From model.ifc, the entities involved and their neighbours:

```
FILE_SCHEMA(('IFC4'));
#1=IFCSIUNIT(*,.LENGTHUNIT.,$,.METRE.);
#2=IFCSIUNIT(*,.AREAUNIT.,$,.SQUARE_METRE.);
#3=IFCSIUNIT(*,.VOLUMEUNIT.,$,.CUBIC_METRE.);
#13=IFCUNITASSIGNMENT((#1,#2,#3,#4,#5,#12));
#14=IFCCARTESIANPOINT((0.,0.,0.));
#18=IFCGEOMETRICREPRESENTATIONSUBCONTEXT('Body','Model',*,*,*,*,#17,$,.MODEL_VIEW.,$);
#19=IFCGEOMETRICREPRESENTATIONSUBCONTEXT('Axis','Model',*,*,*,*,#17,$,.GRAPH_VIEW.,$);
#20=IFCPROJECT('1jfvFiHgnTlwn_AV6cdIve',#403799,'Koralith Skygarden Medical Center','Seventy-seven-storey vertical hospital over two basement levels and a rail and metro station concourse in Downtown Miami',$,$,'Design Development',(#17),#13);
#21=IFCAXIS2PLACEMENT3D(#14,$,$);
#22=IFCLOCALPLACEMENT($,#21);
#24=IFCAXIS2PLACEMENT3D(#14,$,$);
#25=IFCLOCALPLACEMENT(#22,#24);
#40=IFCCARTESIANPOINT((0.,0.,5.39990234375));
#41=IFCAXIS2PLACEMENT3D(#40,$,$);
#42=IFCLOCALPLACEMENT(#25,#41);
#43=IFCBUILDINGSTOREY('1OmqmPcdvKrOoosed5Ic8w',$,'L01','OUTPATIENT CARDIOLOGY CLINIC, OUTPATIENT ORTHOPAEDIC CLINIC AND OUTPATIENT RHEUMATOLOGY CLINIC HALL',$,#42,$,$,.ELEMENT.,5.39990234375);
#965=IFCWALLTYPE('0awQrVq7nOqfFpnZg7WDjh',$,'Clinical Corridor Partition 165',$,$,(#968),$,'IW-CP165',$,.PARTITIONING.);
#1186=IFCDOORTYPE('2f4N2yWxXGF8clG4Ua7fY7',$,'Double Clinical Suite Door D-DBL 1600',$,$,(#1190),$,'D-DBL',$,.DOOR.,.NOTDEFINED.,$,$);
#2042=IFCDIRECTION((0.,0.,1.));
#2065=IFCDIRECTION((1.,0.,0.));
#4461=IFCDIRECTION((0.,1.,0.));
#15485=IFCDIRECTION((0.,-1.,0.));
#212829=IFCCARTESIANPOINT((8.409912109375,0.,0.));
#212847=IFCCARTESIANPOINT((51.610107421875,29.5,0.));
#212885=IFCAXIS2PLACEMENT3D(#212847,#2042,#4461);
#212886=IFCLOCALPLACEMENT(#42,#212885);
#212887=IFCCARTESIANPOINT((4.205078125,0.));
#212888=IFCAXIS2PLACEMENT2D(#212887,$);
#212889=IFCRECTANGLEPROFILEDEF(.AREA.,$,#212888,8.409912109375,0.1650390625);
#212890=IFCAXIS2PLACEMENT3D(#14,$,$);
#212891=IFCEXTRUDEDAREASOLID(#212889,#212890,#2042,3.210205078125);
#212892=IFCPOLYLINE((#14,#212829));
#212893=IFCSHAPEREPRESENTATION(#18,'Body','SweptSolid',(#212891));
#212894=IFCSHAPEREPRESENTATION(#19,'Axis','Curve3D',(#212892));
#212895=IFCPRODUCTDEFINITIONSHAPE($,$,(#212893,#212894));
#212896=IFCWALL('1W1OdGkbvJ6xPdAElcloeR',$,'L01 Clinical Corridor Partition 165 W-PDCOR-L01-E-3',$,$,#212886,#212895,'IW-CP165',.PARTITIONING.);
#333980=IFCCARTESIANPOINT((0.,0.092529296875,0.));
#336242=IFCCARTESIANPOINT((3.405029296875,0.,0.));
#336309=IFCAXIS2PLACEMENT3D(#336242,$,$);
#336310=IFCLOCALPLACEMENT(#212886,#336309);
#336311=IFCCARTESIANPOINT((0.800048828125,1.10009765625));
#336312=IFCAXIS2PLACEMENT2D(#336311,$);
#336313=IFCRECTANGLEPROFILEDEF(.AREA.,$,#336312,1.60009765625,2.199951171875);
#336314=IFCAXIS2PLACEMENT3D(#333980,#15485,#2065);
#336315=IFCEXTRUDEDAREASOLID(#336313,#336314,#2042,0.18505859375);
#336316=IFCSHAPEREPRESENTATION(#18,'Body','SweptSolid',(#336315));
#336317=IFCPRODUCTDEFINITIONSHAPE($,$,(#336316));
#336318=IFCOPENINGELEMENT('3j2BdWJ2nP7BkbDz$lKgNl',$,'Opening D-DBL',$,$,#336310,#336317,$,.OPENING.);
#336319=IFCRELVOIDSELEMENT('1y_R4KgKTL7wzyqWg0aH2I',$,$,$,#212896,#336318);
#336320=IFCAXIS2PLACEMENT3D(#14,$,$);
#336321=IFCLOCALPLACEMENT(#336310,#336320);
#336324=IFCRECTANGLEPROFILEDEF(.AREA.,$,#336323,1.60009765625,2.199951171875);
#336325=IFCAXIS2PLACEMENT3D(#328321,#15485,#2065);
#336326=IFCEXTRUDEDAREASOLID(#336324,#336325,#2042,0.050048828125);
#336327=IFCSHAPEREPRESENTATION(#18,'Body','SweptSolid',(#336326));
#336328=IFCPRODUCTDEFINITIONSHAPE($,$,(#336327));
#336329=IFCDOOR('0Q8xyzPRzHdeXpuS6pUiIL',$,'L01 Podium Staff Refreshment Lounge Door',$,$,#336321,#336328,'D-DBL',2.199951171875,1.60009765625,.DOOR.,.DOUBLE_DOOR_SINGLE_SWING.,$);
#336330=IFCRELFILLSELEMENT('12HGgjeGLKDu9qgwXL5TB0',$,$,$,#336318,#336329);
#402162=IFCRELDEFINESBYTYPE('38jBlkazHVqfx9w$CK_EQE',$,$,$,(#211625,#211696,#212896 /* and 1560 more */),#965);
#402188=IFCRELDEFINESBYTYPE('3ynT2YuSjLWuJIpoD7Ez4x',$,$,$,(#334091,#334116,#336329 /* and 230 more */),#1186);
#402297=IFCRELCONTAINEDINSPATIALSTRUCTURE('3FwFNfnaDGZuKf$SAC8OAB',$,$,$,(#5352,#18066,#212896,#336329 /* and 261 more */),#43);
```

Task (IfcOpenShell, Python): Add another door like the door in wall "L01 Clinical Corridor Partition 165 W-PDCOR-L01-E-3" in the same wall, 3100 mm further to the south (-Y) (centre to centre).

```python
import ifcopenshell
import ifcopenshell.api.feature
import ifcopenshell.api.geometry
import ifcopenshell.api.root
import ifcopenshell.geom
import ifcopenshell.util.element
import ifcopenshell.util.placement
import ifcopenshell.util.shape
import ifcopenshell.util.unit

model = ifcopenshell.open("model.ifc")
unit_scale = ifcopenshell.util.unit.calculate_unit_scale(model)
settings = ifcopenshell.geom.settings()


def volume(element):
    """Net volume in cubic metres, openings subtracted."""
    shape = ifcopenshell.geom.create_shape(settings, element)
    return ifcopenshell.util.shape.get_volume(shape.geometry)


door = model.by_id(336329)
opening = door.FillsVoids[0].RelatingOpeningElement
wall = opening.VoidsElements[0].RelatingBuildingElement
before = volume(wall)
shift = ifcopenshell.util.placement.get_local_placement(wall.ObjectPlacement)[:3, 0] * -3.1 / unit_scale

# copy_class copies the void relationship, type, container and properties, but no geometry.
new_opening = ifcopenshell.api.root.copy_class(model, product=opening)
new_opening.Representation = ifcopenshell.util.element.copy_deep(
    model, opening.Representation, exclude=["IfcGeometricRepresentationContext", "IfcRepresentationMap"]
)
new_door = ifcopenshell.api.root.copy_class(model, product=door)
new_door.Representation = ifcopenshell.util.element.copy_deep(
    model, door.Representation, exclude=["IfcGeometricRepresentationContext", "IfcRepresentationMap"]
)
new_door.Tag = None
ifcopenshell.api.feature.add_filling(model, opening=new_opening, element=new_door)

for old, new in ((opening, new_opening), (door, new_door)):
    matrix = ifcopenshell.util.placement.get_local_placement(old.ObjectPlacement)
    matrix[:3, 3] += shift
    ifcopenshell.api.geometry.edit_object_placement(model, product=new, matrix=matrix, is_si=False)

after = volume(wall)

print(f"wall volume {before:.3f} -> {after:.3f} m3")

model.write("model-out.ifc")
```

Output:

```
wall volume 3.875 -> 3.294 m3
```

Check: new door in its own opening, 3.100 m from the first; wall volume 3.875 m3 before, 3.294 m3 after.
